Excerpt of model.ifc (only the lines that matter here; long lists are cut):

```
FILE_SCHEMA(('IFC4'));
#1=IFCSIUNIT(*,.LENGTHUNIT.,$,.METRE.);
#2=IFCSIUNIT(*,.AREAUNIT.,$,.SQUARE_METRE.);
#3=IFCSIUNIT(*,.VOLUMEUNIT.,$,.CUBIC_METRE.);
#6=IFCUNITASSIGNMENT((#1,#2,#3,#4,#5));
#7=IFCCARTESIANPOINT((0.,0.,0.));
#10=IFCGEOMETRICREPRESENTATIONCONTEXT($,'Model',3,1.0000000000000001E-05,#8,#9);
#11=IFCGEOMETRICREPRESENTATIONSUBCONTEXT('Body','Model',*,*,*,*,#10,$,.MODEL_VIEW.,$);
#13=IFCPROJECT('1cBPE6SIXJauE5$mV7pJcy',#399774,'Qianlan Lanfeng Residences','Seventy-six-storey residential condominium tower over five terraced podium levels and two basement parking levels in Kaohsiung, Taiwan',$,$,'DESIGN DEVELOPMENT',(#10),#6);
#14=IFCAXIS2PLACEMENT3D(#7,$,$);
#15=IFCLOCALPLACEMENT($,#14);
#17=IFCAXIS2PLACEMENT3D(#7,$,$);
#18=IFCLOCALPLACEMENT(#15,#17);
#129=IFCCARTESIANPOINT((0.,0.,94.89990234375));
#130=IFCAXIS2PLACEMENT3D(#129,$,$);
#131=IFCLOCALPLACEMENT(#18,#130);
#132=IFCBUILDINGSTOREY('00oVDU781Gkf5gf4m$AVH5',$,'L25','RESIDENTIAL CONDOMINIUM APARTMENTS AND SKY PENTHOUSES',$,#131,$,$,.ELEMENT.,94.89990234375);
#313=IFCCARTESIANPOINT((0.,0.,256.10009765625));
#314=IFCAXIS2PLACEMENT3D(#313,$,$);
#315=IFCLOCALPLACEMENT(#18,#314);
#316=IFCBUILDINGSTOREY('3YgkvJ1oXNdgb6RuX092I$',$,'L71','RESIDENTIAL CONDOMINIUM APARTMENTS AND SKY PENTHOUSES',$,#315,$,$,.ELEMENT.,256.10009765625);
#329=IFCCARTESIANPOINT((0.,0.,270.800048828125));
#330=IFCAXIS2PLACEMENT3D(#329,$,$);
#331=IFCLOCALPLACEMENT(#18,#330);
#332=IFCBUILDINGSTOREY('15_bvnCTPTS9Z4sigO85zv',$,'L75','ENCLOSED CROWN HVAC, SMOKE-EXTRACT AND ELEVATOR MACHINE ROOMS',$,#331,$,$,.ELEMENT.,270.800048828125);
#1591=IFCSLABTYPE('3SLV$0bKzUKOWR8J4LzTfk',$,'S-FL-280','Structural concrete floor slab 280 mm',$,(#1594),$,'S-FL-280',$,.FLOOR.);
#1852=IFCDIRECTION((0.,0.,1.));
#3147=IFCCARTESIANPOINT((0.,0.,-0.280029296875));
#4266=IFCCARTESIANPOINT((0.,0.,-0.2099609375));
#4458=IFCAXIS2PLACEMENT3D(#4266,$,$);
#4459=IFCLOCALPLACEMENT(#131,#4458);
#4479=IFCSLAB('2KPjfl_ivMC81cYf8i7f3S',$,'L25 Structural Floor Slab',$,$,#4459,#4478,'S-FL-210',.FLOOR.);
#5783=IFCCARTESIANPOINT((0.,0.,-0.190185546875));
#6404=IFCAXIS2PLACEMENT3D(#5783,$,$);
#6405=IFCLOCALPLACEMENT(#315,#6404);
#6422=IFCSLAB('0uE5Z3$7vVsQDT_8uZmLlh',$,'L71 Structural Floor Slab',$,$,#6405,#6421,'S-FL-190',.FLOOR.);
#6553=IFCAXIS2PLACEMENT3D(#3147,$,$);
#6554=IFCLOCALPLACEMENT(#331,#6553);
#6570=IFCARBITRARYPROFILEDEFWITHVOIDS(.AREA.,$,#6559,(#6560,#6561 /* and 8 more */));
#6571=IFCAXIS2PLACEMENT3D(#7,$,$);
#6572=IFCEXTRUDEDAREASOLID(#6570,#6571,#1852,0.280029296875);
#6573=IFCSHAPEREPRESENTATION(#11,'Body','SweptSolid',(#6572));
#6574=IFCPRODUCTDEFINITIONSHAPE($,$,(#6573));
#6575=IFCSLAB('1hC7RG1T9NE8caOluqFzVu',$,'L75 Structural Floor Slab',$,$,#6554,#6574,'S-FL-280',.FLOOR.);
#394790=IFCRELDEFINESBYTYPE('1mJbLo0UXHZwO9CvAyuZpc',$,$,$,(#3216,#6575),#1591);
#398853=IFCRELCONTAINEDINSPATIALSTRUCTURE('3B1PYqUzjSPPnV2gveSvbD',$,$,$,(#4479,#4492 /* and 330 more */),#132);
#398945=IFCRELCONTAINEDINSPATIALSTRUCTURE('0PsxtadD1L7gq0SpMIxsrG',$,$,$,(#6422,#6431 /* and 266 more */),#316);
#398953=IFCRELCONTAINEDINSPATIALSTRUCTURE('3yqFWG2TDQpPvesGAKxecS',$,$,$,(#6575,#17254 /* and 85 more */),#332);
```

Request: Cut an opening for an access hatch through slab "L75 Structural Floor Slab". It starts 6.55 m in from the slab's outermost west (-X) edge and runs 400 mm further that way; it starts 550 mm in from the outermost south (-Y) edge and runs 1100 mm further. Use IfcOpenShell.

```python
import numpy as np
import ifcopenshell
import ifcopenshell.api.feature
import ifcopenshell.api.geometry
import ifcopenshell.api.root
import ifcopenshell.geom
import ifcopenshell.util.placement
import ifcopenshell.util.representation
import ifcopenshell.util.shape
import ifcopenshell.util.unit

model = ifcopenshell.open("model.ifc")
unit_scale = ifcopenshell.util.unit.calculate_unit_scale(model)
settings = ifcopenshell.geom.settings()


def volume(element):
    """Net volume in cubic metres, openings subtracted."""
    shape = ifcopenshell.geom.create_shape(settings, element)
    return ifcopenshell.util.shape.get_volume(shape.geometry)


slab = model.by_id(6575)
before = volume(slab)

# Extent in the slab's own axes, in metres. The edges named are its -X and -Y sides.
slab_shape = ifcopenshell.geom.create_shape(settings, slab)
vertices = ifcopenshell.util.shape.get_vertices(slab_shape.geometry)
x_min, y_min, bottom = vertices.min(axis=0)
top = vertices[:, 2].max()

opening = ifcopenshell.api.root.create_entity(model, ifc_class="IfcOpeningElement", name="Access hatch opening", predefined_type="OPENING")
context = ifcopenshell.util.representation.get_context(model, "Model", "Body", "MODEL_VIEW")
width, depth = 0.4, 1.1
outline = [(0.0, 0.0), (width, 0.0), (width, depth), (0.0, depth), (0.0, 0.0)]
# Overshoot both faces by 50 mm so the cut is clean.
shape = ifcopenshell.api.geometry.add_slab_representation(
    model, context=context, depth=top - bottom + 0.1, polyline=outline
)
ifcopenshell.api.geometry.assign_representation(model, product=opening, representation=shape)

matrix = ifcopenshell.util.placement.get_local_placement(slab.ObjectPlacement)
matrix[:, 3] = matrix @ np.append(np.array([x_min + 6.55, y_min + 0.55, bottom - 0.05]) / unit_scale, 1.0)
ifcopenshell.api.geometry.edit_object_placement(model, product=opening, matrix=matrix, is_si=False)
ifcopenshell.api.feature.add_feature(model, feature=opening, element=slab)

after = volume(slab)

print(f"slab volume {before:.3f} -> {after:.3f} m3")

model.write("model-out.ifc")
```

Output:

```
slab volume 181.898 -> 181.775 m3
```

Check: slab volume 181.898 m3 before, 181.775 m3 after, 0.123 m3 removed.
